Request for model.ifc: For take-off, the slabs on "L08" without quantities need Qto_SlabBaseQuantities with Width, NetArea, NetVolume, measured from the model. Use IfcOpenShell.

First a look at what the model holds.

```python
import ifcopenshell
import ifcopenshell.util.element
import ifcopenshell.util.unit

model = ifcopenshell.open("model.ifc")
print(model.schema)
for unit_type in ("LENGTHUNIT", "AREAUNIT", "VOLUMEUNIT"):
    print(unit_type, ifcopenshell.util.unit.calculate_unit_scale(model, unit_type))
storey = next(s for s in model.by_type("IfcBuildingStorey") if s.Name == "L08")
slabs = [e for e in ifcopenshell.util.element.get_decomposition(storey) if e.is_a("IfcSlab")]
for e in sorted(slabs, key=lambda e: e.id()):
    print(e.id(), e.is_a(), e.Name, list(ifcopenshell.util.element.get_psets(e, qtos_only=True)), sep=" | ")
```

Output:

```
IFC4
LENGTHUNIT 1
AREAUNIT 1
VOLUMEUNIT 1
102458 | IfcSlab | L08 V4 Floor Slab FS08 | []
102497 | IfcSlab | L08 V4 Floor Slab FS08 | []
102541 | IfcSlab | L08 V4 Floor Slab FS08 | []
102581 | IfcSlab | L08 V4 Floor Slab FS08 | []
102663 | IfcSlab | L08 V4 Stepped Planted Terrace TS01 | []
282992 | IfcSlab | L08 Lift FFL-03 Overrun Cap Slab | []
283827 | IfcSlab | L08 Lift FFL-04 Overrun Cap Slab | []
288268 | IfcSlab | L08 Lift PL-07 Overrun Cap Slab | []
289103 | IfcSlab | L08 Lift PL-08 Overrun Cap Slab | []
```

```python
import ifcopenshell
import ifcopenshell.api.pset
import ifcopenshell.geom
import ifcopenshell.util.element
import ifcopenshell.util.shape
import ifcopenshell.util.unit

model = ifcopenshell.open("model.ifc")
unit_scale = ifcopenshell.util.unit.calculate_unit_scale(model)
area_scale = ifcopenshell.util.unit.calculate_unit_scale(model, "AREAUNIT")
volume_scale = ifcopenshell.util.unit.calculate_unit_scale(model, "VOLUMEUNIT")
settings = ifcopenshell.geom.settings()

storey = next(s for s in model.by_type("IfcBuildingStorey") if s.Name == "L08")
slabs = [e for e in ifcopenshell.util.element.get_decomposition(storey) if e.is_a("IfcSlab")]

for e in sorted(slabs, key=lambda e: e.id()):
    if ifcopenshell.util.element.get_psets(e, qtos_only=True, should_inherit=False):
        continue
    # Geometry comes back in metres, in the element's own axes.
    shape = ifcopenshell.geom.create_shape(settings, e)
    values = {
        "Width": ifcopenshell.util.shape.get_z(shape.geometry) / unit_scale,
        "NetArea": ifcopenshell.util.shape.get_footprint_area(shape.geometry) / area_scale,
        "NetVolume": ifcopenshell.util.shape.get_volume(shape.geometry) / volume_scale,
    }
    qto = ifcopenshell.api.pset.add_qto(model, product=e, name="Qto_SlabBaseQuantities")
    ifcopenshell.api.pset.edit_qto(model, qto=qto, properties=values)
    print(e.id(), {k: round(v, 3) for k, v in values.items()})

model.write("model_rev.ifc")
```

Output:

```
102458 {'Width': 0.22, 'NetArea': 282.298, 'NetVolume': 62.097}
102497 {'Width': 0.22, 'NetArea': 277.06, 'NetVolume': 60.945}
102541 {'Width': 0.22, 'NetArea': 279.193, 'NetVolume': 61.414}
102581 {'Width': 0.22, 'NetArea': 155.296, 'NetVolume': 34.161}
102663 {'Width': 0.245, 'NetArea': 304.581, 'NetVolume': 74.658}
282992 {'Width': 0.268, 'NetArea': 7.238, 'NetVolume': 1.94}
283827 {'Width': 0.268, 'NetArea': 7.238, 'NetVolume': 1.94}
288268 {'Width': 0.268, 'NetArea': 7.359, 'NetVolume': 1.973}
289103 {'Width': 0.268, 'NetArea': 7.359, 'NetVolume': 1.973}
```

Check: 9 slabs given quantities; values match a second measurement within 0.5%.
